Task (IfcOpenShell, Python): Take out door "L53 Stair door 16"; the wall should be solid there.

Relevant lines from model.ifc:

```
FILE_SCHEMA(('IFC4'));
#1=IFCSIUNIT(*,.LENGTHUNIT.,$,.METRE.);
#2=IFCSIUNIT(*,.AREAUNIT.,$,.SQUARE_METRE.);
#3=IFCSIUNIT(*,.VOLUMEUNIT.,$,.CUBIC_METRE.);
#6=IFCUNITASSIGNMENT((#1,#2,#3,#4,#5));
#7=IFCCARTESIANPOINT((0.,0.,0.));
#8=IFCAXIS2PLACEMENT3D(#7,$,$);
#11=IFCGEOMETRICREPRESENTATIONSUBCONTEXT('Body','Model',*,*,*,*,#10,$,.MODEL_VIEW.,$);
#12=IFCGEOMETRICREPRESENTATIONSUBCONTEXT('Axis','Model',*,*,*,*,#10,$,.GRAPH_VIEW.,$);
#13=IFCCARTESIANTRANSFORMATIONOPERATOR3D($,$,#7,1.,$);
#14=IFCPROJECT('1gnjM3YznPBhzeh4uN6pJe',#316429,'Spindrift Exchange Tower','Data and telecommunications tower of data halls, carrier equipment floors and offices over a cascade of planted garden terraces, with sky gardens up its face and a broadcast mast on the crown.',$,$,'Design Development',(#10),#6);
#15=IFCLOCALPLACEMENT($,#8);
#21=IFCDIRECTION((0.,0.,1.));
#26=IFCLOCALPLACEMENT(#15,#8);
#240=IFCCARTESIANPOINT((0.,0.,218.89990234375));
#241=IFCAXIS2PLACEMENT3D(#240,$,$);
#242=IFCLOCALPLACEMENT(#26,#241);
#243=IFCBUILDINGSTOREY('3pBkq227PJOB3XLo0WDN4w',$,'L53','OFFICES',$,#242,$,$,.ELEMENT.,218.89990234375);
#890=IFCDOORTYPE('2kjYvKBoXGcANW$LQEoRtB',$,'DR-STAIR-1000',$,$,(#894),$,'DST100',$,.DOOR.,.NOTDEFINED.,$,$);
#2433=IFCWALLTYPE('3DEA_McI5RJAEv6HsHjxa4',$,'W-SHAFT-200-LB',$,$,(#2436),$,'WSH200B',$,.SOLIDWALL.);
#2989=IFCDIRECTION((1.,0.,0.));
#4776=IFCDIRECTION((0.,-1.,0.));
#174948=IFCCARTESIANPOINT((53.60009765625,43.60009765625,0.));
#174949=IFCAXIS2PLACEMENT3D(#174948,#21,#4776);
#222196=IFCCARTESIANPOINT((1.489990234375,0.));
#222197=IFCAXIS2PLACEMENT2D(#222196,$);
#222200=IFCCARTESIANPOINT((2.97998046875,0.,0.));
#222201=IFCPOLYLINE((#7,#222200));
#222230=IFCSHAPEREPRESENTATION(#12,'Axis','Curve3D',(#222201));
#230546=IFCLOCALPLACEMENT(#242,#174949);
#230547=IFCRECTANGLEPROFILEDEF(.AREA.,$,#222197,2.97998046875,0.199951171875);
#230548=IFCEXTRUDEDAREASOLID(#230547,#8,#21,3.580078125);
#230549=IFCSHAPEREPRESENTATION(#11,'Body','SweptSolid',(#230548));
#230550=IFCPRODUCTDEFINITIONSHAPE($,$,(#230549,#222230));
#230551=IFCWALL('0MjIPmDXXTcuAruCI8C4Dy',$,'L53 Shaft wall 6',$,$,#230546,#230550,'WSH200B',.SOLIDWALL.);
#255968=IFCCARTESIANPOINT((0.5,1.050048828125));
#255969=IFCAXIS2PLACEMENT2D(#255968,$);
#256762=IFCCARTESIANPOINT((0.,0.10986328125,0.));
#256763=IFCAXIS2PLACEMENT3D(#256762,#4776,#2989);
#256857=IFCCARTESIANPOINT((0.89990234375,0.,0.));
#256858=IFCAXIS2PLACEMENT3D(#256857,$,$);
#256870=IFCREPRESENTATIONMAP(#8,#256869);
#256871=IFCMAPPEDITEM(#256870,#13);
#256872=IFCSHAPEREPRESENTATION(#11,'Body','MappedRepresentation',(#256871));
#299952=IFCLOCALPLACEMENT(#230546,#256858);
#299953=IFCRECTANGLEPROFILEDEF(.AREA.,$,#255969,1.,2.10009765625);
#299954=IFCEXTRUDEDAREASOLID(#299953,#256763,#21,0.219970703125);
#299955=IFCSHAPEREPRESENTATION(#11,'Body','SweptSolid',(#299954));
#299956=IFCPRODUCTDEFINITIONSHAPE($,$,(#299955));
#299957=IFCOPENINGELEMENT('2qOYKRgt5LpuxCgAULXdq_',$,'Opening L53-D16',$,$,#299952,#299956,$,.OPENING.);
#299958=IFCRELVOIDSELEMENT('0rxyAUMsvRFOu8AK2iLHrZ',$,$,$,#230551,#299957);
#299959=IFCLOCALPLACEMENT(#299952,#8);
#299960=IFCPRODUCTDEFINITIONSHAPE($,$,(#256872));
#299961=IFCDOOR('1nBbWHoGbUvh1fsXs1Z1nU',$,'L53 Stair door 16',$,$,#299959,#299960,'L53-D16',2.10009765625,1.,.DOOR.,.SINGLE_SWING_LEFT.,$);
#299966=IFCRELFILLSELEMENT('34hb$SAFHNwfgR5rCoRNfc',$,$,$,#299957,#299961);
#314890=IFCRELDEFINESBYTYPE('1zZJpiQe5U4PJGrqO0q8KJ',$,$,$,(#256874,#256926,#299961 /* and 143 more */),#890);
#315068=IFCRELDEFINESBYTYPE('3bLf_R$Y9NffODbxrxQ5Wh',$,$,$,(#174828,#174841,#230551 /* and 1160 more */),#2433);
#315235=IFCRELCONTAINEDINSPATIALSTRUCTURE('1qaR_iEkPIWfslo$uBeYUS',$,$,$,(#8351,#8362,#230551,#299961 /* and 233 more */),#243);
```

```python
import ifcopenshell
import ifcopenshell.api.feature
import ifcopenshell.api.root
import ifcopenshell.geom
import ifcopenshell.util.shape

model = ifcopenshell.open("model.ifc")
settings = ifcopenshell.geom.settings()


def volume(element):
    """Net volume in cubic metres, openings subtracted."""
    shape = ifcopenshell.geom.create_shape(settings, element)
    return ifcopenshell.util.shape.get_volume(shape.geometry)


door = model.by_guid("1nBbWHoGbUvh1fsXs1Z1nU")
opening = door.FillsVoids[0].RelatingOpeningElement
wall = opening.VoidsElements[0].RelatingBuildingElement
before = volume(wall)

ifcopenshell.api.root.remove_product(model, product=door)
ifcopenshell.api.feature.remove_feature(model, feature=opening)

after = volume(wall)

print(f"wall volume {before:.3f} -> {after:.3f} m3")

model.write("model_v2.ifc")
```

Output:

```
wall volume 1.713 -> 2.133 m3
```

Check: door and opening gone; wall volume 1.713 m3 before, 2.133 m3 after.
